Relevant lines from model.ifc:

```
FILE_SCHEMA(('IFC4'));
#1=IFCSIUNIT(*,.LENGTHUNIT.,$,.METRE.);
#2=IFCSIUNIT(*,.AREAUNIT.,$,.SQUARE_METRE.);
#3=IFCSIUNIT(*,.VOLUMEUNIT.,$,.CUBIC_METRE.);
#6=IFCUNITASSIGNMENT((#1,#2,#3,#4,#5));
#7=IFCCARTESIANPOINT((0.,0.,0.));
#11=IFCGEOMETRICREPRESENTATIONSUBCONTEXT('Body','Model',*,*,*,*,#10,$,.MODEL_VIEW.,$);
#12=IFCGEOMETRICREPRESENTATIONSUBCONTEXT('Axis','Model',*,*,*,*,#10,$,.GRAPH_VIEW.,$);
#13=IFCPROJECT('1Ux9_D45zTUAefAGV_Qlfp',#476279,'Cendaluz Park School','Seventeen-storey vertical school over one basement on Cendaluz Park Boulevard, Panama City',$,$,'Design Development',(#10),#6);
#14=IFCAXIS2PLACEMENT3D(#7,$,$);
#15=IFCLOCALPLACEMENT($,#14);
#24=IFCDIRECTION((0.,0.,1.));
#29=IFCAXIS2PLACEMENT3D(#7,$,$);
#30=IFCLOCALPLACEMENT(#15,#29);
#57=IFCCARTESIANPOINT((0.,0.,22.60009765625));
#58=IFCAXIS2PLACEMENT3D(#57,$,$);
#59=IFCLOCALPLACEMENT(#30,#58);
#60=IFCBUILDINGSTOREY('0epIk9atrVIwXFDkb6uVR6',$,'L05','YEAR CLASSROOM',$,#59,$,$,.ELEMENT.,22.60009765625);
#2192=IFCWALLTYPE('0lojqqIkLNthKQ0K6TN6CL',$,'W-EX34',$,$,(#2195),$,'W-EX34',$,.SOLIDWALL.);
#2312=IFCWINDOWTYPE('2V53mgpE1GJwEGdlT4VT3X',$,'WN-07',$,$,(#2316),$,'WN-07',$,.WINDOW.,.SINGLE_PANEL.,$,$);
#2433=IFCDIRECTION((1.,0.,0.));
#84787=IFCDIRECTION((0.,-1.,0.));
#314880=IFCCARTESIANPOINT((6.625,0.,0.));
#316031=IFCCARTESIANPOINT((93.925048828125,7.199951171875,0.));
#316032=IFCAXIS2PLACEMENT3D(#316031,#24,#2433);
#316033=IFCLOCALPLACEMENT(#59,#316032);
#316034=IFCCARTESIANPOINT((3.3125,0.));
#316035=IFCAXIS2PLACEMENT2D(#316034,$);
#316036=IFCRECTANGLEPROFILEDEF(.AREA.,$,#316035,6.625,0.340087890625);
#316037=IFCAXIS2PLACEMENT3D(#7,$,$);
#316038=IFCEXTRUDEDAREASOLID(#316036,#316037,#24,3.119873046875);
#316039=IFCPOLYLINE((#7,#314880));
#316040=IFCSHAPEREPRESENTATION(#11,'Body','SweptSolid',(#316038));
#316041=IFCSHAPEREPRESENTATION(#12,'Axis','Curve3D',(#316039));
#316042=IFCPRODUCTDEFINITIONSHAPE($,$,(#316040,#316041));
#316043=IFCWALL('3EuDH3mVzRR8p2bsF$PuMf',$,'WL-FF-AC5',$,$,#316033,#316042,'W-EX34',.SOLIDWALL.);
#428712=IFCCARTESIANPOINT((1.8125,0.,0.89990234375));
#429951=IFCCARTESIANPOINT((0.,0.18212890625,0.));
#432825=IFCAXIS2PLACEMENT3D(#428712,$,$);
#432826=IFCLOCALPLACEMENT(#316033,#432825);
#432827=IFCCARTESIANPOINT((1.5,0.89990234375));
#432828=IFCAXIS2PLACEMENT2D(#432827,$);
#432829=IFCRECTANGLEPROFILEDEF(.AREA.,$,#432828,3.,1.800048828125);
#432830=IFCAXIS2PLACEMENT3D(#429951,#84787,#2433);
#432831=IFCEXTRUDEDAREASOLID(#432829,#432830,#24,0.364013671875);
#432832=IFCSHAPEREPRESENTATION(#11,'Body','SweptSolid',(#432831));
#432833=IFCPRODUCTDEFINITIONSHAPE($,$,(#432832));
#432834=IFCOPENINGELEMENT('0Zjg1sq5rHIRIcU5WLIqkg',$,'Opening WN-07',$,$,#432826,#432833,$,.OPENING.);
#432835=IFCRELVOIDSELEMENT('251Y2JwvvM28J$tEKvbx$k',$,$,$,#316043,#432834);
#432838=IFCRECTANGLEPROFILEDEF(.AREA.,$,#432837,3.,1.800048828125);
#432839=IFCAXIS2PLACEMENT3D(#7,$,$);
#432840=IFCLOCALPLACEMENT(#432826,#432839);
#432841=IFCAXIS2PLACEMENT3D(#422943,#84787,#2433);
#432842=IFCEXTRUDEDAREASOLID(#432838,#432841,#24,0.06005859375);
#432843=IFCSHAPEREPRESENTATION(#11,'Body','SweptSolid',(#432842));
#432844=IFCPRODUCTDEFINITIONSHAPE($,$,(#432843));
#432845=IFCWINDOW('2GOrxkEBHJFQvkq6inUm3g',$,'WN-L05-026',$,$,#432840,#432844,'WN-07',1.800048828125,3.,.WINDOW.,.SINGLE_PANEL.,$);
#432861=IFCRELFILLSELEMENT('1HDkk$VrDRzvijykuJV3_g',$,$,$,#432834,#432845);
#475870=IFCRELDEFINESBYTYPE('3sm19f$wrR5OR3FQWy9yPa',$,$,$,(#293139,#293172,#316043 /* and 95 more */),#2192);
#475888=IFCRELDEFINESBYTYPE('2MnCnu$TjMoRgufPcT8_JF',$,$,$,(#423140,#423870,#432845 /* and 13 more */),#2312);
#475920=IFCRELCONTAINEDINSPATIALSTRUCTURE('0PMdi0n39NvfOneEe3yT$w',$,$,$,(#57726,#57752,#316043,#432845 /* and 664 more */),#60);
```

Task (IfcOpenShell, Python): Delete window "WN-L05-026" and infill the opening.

```python
import ifcopenshell
import ifcopenshell.api.feature
import ifcopenshell.api.root
import ifcopenshell.geom
import ifcopenshell.util.shape

model = ifcopenshell.open("model.ifc")
settings = ifcopenshell.geom.settings()


def volume(element):
    """Net volume in cubic metres, openings subtracted."""
    shape = ifcopenshell.geom.create_shape(settings, element)
    return ifcopenshell.util.shape.get_volume(shape.geometry)


window = model.by_guid("2GOrxkEBHJFQvkq6inUm3g")
opening = window.FillsVoids[0].RelatingOpeningElement
wall = opening.VoidsElements[0].RelatingBuildingElement
before = volume(wall)

ifcopenshell.api.root.remove_product(model, product=window)
ifcopenshell.api.feature.remove_feature(model, feature=opening)

after = volume(wall)

print(f"wall volume {before:.3f} -> {after:.3f} m3")

model.write("model_v2.ifc")
```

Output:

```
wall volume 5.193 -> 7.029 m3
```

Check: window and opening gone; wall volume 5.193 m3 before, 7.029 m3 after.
